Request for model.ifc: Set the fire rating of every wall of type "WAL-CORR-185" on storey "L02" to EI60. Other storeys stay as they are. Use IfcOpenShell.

First a look at what the model holds.

```python
import ifcopenshell
import ifcopenshell.util.element

model = ifcopenshell.open("model.ifc")
print(model.schema)
storey = next(s for s in model.by_type("IfcBuildingStorey") if s.Name == "L02")
walls = [e for e in ifcopenshell.util.element.get_decomposition(storey) if e.is_a("IfcWall")]
seen = {}
for e in walls:
    element_type = ifcopenshell.util.element.get_type(e)
    key = (element_type.Name if element_type != e and element_type else None, ifcopenshell.util.element.get_pset(e, "Pset_WallCommon", "FireRating"))
    seen[key] = seen.get(key, 0) + 1
for (name, value), count in sorted(seen.items(), key=str):
    print(count, "x", name, "|", value)
```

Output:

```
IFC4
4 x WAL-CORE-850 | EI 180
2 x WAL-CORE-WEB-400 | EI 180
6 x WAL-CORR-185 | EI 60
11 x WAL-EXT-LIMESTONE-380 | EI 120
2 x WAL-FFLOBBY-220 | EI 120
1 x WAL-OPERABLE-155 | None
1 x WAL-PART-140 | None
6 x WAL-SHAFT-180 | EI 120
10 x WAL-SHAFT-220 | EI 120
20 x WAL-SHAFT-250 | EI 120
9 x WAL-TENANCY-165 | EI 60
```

```python
import ifcopenshell
import ifcopenshell.api.pset
import ifcopenshell.util.element

model = ifcopenshell.open("model.ifc")

storey = next(s for s in model.by_type("IfcBuildingStorey") if s.Name == "L02")
walls = [e for e in ifcopenshell.util.element.get_decomposition(storey) if e.is_a("IfcWall")]

count = 0
for e in walls:
    element_type = ifcopenshell.util.element.get_type(e)
    if element_type in (None, e) or element_type.Name != "WAL-CORR-185":
        continue
    found = ifcopenshell.util.element.get_pset(e, "Pset_WallCommon", should_inherit=False)
    if found:
        pset = model.by_id(found["id"])
        if len(ifcopenshell.util.element.get_elements_by_pset(pset)) > 1:
            pset = ifcopenshell.api.pset.unshare_pset(model, products=[e], pset=pset)[0]
    else:
        pset = ifcopenshell.api.pset.add_pset(model, product=e, name="Pset_WallCommon")
    ifcopenshell.api.pset.edit_pset(model, pset=pset, properties={"FireRating": "EI60"})
    count += 1

print(count, "walls updated")

model.write("model_v2.ifc")
```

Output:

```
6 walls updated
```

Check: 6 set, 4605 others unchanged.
